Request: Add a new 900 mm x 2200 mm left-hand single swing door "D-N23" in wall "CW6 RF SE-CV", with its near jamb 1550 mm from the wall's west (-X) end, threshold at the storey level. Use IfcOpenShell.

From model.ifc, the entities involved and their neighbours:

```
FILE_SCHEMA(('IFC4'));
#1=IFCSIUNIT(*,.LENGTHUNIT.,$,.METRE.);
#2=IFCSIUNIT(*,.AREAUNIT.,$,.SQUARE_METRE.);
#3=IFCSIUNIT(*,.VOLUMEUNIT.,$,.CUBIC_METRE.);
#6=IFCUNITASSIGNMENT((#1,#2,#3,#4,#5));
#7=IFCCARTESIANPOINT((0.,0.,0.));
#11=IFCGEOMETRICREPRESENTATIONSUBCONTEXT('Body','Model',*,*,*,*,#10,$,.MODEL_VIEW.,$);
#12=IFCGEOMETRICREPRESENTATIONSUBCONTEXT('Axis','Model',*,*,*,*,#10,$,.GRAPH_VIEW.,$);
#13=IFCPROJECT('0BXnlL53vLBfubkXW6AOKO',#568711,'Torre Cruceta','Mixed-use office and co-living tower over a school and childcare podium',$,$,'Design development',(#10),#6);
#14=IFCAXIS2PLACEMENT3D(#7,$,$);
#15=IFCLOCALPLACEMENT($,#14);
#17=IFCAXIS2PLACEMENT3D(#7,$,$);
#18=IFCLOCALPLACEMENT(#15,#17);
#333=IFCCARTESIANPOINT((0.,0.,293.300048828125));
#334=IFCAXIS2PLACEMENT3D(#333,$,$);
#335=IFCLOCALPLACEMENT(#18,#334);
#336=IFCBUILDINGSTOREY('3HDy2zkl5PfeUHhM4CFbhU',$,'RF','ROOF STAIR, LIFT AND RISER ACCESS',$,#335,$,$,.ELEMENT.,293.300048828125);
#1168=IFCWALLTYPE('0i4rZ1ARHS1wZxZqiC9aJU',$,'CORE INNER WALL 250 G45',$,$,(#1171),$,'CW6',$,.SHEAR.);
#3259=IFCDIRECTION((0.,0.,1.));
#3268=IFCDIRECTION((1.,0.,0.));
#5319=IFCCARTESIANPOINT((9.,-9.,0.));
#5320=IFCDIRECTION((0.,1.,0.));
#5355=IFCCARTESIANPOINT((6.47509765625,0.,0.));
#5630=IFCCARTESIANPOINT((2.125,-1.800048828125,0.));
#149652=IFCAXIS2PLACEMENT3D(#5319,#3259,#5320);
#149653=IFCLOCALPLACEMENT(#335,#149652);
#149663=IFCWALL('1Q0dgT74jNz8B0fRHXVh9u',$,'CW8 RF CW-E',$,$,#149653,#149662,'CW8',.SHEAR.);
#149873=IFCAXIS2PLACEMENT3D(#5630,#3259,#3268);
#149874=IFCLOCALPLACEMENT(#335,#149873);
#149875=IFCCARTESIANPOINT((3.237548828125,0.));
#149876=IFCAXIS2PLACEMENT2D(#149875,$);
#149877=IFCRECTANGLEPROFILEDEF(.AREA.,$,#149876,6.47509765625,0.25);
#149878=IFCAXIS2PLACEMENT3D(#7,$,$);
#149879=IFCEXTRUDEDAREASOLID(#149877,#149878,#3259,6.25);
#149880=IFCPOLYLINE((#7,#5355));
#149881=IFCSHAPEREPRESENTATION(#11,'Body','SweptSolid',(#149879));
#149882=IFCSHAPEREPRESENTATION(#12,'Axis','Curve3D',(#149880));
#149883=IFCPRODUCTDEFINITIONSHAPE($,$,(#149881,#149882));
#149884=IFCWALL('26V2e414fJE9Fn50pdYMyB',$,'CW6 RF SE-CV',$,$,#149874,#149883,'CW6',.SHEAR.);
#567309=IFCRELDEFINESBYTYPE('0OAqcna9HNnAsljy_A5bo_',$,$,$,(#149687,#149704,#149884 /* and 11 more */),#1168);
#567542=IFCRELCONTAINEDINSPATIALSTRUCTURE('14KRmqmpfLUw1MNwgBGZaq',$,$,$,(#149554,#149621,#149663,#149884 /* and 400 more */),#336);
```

```python
import numpy as np
import ifcopenshell
import ifcopenshell.api.feature
import ifcopenshell.api.geometry
import ifcopenshell.api.root
import ifcopenshell.api.spatial
import ifcopenshell.geom
import ifcopenshell.util.element
import ifcopenshell.util.placement
import ifcopenshell.util.representation
import ifcopenshell.util.shape
import ifcopenshell.util.unit

model = ifcopenshell.open("model.ifc")
unit_scale = ifcopenshell.util.unit.calculate_unit_scale(model)
settings = ifcopenshell.geom.settings()


def volume(element):
    """Net volume in cubic metres, openings subtracted."""
    shape = ifcopenshell.geom.create_shape(settings, element)
    return ifcopenshell.util.shape.get_volume(shape.geometry)


wall = model.by_guid("26V2e414fJE9Fn50pdYMyB")
storey = ifcopenshell.util.element.get_container(wall, ifc_class="IfcBuildingStorey")
context = ifcopenshell.util.representation.get_context(model, "Model", "Body", "MODEL_VIEW")
before = volume(wall)

width, height, from_end, sill = 0.9, 2.2, 1.55, 0.0  # metres

# The wall runs along its own X axis, and the end named is its -X end.
wall_shape = ifcopenshell.geom.create_shape(settings, wall)
x, y, z = ifcopenshell.util.shape.get_vertices(wall_shape.geometry).T
start = x.min() + from_end
face, thickness = float(y.min()), float(y.max() - y.min())
wall_matrix = ifcopenshell.util.placement.get_local_placement(wall.ObjectPlacement)
level = ifcopenshell.util.placement.get_local_placement(storey.ObjectPlacement)[2, 3]


def in_wall(x, y):
    """Placement at x, y metres in the wall's axes, at sill height."""
    matrix = wall_matrix.copy()
    matrix[:, 3] = wall_matrix @ np.array([x / unit_scale, y / unit_scale, 0.0, 1.0])
    matrix[2, 3] = level + sill / unit_scale
    return matrix


# Opening: a box that overshoots both wall faces by 50 mm.
opening = ifcopenshell.api.root.create_entity(model, ifc_class="IfcOpeningElement", predefined_type="OPENING")
box = ifcopenshell.api.geometry.add_wall_representation(
    model, context=context, length=width, height=height, thickness=thickness + 0.1
)
ifcopenshell.api.geometry.assign_representation(model, product=opening, representation=box)
ifcopenshell.api.geometry.edit_object_placement(model, product=opening, matrix=in_wall(start, face - 0.05), is_si=False)
ifcopenshell.api.feature.add_feature(model, feature=opening, element=wall)

door = ifcopenshell.api.root.create_entity(model, ifc_class="IfcDoor", name="D-N23", predefined_type="DOOR")
door.OverallWidth, door.OverallHeight = width / unit_scale, height / unit_scale
door.OperationType = "SINGLE_SWING_LEFT"
body = ifcopenshell.api.geometry.add_door_representation(
    model,
    context=context,
    overall_width=door.OverallWidth,
    overall_height=door.OverallHeight,
    operation_type="SINGLE_SWING_LEFT",
    lining_properties={"LiningDepth": thickness / unit_scale, "ThresholdDepth": thickness / unit_scale},
)
ifcopenshell.api.geometry.assign_representation(model, product=door, representation=body)
ifcopenshell.api.spatial.assign_container(model, products=[door], relating_structure=storey)
ifcopenshell.api.feature.add_filling(model, opening=opening, element=door)

# The lining spans the wall, so the door starts at the wall face.
ifcopenshell.api.geometry.edit_object_placement(model, product=door, matrix=in_wall(start, face), is_si=False)

after = volume(wall)

print(f"wall volume {before:.3f} -> {after:.3f} m3")

model.write("model_rev.ifc")
```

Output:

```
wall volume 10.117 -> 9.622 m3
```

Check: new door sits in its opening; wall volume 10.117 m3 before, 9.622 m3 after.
